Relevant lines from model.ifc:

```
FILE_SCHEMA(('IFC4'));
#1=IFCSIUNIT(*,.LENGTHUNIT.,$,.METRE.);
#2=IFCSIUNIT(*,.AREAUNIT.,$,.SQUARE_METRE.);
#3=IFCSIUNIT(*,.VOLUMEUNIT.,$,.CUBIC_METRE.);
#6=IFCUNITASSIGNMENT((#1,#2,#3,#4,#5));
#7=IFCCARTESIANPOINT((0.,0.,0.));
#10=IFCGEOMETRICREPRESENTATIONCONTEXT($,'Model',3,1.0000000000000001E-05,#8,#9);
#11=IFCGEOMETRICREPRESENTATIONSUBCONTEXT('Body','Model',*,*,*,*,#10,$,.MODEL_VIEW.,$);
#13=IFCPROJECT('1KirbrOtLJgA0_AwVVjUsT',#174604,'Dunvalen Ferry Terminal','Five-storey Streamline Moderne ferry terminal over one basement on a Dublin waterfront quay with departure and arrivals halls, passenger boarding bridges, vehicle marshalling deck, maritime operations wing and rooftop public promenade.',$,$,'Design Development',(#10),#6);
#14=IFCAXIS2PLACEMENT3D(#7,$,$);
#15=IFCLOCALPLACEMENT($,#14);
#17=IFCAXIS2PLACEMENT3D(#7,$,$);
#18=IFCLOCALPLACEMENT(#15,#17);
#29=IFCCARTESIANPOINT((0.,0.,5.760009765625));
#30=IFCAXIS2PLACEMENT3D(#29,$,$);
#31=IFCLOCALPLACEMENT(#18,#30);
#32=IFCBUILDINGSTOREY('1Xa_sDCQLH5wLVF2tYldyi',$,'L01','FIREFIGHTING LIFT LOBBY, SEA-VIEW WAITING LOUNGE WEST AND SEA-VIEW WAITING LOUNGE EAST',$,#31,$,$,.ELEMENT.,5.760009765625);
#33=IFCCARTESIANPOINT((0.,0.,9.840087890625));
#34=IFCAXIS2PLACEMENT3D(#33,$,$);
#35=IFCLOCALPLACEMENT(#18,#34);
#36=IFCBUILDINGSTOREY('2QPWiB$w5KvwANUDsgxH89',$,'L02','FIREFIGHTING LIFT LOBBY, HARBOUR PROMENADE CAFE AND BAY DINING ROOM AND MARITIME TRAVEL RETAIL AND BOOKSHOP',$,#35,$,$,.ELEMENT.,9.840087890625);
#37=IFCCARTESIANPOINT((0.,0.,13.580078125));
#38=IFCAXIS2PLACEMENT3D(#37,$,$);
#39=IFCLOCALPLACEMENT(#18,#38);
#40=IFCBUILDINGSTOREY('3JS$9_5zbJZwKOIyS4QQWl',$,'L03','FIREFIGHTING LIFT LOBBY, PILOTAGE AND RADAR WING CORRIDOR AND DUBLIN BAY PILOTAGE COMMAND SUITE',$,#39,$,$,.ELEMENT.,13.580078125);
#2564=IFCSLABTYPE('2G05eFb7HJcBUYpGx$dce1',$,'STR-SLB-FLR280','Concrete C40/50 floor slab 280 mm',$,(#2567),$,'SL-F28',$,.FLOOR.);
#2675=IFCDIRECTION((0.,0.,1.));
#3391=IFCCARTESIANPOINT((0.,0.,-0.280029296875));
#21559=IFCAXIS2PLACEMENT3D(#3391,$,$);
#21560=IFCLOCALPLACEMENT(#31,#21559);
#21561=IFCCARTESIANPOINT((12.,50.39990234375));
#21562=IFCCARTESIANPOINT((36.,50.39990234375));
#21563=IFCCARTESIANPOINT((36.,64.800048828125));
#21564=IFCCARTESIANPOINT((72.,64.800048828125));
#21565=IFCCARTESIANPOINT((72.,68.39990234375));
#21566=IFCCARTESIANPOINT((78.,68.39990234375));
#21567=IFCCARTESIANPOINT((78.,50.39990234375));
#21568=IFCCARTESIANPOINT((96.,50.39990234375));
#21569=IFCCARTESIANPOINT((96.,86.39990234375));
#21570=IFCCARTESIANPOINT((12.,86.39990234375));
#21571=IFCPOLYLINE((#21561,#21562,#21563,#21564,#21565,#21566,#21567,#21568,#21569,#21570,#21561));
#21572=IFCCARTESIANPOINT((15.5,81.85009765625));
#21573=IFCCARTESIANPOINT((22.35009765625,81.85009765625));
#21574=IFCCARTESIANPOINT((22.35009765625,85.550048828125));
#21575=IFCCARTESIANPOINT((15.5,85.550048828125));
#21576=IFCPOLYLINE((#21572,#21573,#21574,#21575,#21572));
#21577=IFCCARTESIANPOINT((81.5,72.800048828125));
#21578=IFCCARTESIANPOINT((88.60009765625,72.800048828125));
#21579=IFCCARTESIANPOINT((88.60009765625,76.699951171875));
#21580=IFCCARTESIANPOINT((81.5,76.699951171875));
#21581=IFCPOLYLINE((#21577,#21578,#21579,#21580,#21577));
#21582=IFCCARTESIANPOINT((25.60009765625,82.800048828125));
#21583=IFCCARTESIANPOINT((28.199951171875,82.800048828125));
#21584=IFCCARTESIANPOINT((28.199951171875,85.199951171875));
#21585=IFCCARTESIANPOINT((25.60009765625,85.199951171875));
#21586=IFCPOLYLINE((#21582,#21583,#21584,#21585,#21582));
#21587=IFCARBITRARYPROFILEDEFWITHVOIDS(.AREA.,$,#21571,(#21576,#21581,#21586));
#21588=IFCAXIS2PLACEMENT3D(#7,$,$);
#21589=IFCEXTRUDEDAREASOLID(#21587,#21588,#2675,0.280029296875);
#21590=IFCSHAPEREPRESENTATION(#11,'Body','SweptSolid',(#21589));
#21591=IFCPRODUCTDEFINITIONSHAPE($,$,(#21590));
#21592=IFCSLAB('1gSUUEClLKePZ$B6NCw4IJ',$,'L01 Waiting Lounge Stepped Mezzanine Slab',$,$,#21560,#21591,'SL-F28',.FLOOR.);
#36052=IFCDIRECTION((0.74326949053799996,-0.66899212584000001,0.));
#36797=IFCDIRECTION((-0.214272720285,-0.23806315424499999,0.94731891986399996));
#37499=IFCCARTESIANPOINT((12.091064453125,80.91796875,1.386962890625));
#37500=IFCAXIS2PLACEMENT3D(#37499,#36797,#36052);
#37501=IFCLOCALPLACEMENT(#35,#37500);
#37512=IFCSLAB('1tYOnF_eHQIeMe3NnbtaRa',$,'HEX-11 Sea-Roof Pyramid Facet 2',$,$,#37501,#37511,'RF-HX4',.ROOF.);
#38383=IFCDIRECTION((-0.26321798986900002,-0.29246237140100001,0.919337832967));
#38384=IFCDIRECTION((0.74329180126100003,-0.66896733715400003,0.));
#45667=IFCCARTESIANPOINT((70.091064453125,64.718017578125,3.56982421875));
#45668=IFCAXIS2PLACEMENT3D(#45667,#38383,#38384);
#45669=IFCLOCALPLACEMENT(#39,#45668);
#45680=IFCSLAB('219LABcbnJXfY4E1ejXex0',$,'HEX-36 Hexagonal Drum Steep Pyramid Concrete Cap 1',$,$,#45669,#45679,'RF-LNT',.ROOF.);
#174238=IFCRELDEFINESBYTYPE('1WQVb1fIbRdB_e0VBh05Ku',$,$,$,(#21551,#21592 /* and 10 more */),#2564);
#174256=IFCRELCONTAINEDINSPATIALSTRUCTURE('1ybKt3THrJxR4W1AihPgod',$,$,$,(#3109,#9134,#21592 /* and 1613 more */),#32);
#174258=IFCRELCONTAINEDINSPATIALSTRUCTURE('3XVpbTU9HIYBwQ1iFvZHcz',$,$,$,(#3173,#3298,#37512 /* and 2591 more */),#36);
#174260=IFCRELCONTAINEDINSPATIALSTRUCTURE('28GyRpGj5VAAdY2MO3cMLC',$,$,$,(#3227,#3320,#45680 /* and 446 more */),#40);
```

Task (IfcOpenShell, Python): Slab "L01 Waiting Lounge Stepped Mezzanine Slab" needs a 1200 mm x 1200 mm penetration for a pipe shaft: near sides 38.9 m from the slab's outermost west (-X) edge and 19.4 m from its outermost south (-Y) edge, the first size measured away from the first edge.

```python
import numpy as np
import ifcopenshell
import ifcopenshell.api.feature
import ifcopenshell.api.geometry
import ifcopenshell.api.root
import ifcopenshell.geom
import ifcopenshell.util.placement
import ifcopenshell.util.representation
import ifcopenshell.util.shape
import ifcopenshell.util.unit

model = ifcopenshell.open("model.ifc")
unit_scale = ifcopenshell.util.unit.calculate_unit_scale(model)
settings = ifcopenshell.geom.settings()


def volume(element):
    """Net volume in cubic metres, openings subtracted."""
    shape = ifcopenshell.geom.create_shape(settings, element)
    return ifcopenshell.util.shape.get_volume(shape.geometry)


slab = model.by_guid("1gSUUEClLKePZ$B6NCw4IJ")
before = volume(slab)

# Extent in the slab's own axes, in metres. The edges named are its -X and -Y sides.
slab_shape = ifcopenshell.geom.create_shape(settings, slab)
vertices = ifcopenshell.util.shape.get_vertices(slab_shape.geometry)
x_min, y_min, bottom = vertices.min(axis=0)
top = vertices[:, 2].max()

opening = ifcopenshell.api.root.create_entity(model, ifc_class="IfcOpeningElement", name="Pipe shaft opening", predefined_type="OPENING")
context = ifcopenshell.util.representation.get_context(model, "Model", "Body", "MODEL_VIEW")
width, depth = 1.2, 1.2
outline = [(0.0, 0.0), (width, 0.0), (width, depth), (0.0, depth), (0.0, 0.0)]
# Overshoot both faces by 50 mm so the cut is clean.
shape = ifcopenshell.api.geometry.add_slab_representation(
    model, context=context, depth=top - bottom + 0.1, polyline=outline
)
ifcopenshell.api.geometry.assign_representation(model, product=opening, representation=shape)

matrix = ifcopenshell.util.placement.get_local_placement(slab.ObjectPlacement)
matrix[:, 3] = matrix @ np.append(np.array([x_min + 38.9, y_min + 19.4, bottom - 0.05]) / unit_scale, 1.0)
ifcopenshell.api.geometry.edit_object_placement(model, product=opening, matrix=matrix, is_si=False)
ifcopenshell.api.feature.add_feature(model, feature=opening, element=slab)

after = volume(slab)

print(f"slab volume {before:.3f} -> {after:.3f} m3")

model.write("model-out.ifc")
```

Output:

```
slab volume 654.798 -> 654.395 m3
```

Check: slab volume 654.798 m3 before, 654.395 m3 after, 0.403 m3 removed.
